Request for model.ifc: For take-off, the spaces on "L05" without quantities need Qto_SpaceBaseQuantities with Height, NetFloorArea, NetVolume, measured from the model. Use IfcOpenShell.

First a look at what the model holds.

```python
import ifcopenshell
import ifcopenshell.util.element
import ifcopenshell.util.unit

model = ifcopenshell.open("model.ifc")
print(model.schema)
for unit_type in ("LENGTHUNIT", "AREAUNIT", "VOLUMEUNIT"):
    print(unit_type, ifcopenshell.util.unit.calculate_unit_scale(model, unit_type))
storey = next(s for s in model.by_type("IfcBuildingStorey") if s.Name == "L05")
spaces = [e for e in ifcopenshell.util.element.get_decomposition(storey) if e.is_a("IfcSpace")]
for e in sorted(spaces, key=lambda e: e.id()):
    print(e.id(), e.is_a(), e.Name, list(ifcopenshell.util.element.get_psets(e, qtos_only=True)), sep=" | ")
```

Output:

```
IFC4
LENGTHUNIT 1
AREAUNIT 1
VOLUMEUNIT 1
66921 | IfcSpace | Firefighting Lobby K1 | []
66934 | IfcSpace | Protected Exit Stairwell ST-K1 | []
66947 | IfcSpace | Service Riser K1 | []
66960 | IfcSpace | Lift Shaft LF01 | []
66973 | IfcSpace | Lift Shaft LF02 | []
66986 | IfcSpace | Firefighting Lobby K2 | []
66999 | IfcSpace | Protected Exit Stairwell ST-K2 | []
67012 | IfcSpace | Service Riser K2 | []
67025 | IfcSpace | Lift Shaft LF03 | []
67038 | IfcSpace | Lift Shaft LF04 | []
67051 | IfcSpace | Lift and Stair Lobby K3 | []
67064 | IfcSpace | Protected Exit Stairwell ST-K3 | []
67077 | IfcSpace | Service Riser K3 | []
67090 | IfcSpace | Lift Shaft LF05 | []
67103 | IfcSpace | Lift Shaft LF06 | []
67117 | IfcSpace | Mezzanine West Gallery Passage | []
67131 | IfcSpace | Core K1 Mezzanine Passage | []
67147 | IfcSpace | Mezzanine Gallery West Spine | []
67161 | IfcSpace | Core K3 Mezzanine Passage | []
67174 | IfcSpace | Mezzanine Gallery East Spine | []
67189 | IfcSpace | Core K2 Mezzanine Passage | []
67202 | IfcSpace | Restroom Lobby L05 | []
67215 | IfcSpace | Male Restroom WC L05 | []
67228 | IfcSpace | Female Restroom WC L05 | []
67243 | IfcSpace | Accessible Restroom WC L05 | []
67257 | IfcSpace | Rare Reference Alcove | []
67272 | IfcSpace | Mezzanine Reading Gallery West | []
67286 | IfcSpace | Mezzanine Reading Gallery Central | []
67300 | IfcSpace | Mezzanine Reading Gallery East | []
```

```python
import ifcopenshell
import ifcopenshell.api.pset
import ifcopenshell.geom
import ifcopenshell.util.element
import ifcopenshell.util.shape
import ifcopenshell.util.unit

model = ifcopenshell.open("model.ifc")
unit_scale = ifcopenshell.util.unit.calculate_unit_scale(model)
area_scale = ifcopenshell.util.unit.calculate_unit_scale(model, "AREAUNIT")
volume_scale = ifcopenshell.util.unit.calculate_unit_scale(model, "VOLUMEUNIT")
settings = ifcopenshell.geom.settings()

storey = next(s for s in model.by_type("IfcBuildingStorey") if s.Name == "L05")
spaces = [e for e in ifcopenshell.util.element.get_decomposition(storey) if e.is_a("IfcSpace")]

for e in sorted(spaces, key=lambda e: e.id()):
    if ifcopenshell.util.element.get_psets(e, qtos_only=True, should_inherit=False):
        continue
    # Geometry comes back in metres, in the element's own axes.
    shape = ifcopenshell.geom.create_shape(settings, e)
    values = {
        "Height": ifcopenshell.util.shape.get_z(shape.geometry) / unit_scale,
        "NetFloorArea": ifcopenshell.util.shape.get_footprint_area(shape.geometry) / area_scale,
        "NetVolume": ifcopenshell.util.shape.get_volume(shape.geometry) / volume_scale,
    }
    qto = ifcopenshell.api.pset.add_qto(model, product=e, name="Qto_SpaceBaseQuantities")
    ifcopenshell.api.pset.edit_qto(model, qto=qto, properties=values)
    print(e.id(), {k: round(v, 3) for k, v in values.items()})

model.write("model_v2.ifc")
```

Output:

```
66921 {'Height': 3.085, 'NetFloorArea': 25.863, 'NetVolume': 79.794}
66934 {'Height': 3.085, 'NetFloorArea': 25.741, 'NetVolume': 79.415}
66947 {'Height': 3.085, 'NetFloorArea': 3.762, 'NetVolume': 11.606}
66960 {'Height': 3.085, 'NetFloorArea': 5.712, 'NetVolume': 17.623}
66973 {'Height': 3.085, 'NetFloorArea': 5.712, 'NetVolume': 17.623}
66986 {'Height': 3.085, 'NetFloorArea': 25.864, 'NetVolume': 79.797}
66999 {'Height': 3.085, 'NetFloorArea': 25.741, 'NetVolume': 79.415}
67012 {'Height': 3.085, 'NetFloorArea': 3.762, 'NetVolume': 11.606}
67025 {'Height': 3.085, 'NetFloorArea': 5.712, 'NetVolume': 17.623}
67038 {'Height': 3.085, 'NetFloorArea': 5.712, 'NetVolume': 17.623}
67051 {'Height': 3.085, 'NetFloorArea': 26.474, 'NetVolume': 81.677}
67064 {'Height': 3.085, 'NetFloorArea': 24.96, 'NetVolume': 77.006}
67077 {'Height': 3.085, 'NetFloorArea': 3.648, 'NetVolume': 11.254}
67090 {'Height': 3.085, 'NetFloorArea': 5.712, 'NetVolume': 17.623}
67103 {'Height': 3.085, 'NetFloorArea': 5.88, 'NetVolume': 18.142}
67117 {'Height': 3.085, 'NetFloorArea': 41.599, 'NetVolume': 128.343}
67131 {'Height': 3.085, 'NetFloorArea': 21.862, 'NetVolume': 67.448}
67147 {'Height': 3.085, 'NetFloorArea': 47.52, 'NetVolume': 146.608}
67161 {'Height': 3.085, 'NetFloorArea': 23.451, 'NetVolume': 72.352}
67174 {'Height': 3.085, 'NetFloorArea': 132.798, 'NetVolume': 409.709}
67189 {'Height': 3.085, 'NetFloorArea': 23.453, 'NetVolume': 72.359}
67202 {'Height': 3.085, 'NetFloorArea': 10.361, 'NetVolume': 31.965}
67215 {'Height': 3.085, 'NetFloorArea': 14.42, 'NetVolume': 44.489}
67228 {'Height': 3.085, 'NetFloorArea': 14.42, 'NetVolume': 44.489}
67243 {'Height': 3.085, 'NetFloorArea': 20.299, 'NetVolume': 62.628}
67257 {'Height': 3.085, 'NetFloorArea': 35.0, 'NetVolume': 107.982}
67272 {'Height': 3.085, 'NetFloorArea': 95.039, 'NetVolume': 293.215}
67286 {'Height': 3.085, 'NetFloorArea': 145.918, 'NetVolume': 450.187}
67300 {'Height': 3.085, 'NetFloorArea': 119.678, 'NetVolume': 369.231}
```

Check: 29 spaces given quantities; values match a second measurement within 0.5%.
